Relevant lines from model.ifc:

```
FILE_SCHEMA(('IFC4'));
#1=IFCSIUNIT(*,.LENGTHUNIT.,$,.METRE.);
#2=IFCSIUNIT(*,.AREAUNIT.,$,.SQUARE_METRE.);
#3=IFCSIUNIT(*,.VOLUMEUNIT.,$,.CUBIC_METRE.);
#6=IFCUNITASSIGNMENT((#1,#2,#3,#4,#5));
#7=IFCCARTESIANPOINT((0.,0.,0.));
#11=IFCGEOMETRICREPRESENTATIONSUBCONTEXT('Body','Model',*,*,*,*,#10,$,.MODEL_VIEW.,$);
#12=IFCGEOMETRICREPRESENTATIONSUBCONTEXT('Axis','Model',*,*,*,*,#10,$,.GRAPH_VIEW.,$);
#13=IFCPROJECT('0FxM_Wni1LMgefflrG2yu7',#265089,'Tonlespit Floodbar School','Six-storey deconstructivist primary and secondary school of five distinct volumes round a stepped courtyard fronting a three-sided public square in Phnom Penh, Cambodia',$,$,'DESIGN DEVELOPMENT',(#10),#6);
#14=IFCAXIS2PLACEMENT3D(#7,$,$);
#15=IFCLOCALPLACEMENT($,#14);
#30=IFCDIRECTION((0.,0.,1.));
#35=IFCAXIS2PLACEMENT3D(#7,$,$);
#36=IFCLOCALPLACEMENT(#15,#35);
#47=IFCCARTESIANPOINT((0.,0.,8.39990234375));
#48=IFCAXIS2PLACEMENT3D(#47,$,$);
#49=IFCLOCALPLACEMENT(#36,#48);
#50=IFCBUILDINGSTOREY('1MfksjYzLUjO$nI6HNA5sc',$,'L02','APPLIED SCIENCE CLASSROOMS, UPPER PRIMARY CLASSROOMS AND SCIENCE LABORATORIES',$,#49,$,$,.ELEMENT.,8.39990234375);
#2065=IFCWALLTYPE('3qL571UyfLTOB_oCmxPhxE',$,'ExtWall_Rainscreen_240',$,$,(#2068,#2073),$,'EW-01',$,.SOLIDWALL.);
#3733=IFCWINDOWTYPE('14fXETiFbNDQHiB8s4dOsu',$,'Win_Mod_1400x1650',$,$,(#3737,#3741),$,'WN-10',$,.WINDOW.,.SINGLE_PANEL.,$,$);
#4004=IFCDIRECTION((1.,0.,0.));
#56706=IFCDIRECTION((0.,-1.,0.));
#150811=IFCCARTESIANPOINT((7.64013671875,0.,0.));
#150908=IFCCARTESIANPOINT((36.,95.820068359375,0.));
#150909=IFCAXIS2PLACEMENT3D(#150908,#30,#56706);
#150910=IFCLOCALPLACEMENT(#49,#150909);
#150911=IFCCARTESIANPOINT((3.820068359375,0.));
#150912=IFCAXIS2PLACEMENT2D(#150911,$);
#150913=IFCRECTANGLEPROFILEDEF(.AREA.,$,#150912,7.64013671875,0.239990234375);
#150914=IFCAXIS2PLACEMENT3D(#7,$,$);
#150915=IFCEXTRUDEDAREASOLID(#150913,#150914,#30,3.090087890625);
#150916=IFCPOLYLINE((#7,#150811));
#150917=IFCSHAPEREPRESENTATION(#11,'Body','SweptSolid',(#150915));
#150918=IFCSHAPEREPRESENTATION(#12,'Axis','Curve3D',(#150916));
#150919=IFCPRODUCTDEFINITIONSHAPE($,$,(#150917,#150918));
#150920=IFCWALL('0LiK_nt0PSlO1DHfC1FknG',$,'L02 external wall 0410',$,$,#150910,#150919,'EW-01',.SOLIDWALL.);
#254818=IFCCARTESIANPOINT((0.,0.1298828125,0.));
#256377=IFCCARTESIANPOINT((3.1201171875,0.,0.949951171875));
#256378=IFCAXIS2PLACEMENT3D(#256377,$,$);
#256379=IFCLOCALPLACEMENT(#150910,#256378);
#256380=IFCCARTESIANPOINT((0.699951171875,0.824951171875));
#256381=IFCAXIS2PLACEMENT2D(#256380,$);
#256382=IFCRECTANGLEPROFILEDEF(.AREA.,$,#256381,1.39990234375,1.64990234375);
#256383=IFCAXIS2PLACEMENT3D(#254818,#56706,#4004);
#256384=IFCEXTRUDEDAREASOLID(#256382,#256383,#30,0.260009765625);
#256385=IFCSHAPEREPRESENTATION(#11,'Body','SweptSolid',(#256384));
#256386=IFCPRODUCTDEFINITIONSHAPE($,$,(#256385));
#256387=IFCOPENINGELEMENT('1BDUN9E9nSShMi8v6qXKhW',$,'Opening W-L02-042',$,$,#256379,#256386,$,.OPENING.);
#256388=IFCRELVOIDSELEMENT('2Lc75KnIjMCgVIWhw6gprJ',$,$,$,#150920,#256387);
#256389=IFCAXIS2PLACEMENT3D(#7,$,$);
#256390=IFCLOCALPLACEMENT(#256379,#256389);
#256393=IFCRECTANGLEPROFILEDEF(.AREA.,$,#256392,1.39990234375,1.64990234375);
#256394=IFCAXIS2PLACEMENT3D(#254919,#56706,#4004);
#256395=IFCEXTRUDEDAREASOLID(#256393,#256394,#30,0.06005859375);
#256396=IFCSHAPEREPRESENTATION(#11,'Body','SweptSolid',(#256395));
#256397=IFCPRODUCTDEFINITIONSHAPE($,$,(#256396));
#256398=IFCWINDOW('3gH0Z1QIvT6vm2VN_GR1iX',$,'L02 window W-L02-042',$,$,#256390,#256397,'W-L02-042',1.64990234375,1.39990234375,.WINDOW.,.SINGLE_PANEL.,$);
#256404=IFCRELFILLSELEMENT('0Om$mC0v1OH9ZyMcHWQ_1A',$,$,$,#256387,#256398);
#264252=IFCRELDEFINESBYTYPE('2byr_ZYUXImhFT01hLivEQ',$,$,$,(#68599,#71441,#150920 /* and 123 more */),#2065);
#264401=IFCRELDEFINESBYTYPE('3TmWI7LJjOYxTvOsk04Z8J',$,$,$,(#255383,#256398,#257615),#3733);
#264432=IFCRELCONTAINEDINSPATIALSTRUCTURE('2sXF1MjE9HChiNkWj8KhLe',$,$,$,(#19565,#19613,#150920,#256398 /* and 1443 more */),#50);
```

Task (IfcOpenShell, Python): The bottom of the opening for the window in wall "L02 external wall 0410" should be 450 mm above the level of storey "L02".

```python
import numpy as np
import ifcopenshell
import ifcopenshell.api.geometry
import ifcopenshell.geom
import ifcopenshell.util.element
import ifcopenshell.util.placement
import ifcopenshell.util.shape
import ifcopenshell.util.unit

model = ifcopenshell.open("model.ifc")
unit_scale = ifcopenshell.util.unit.calculate_unit_scale(model)

window = model.by_guid("3gH0Z1QIvT6vm2VN_GR1iX")
opening = window.FillsVoids[0].RelatingOpeningElement
storey = ifcopenshell.util.element.get_container(window, ifc_class="IfcBuildingStorey")
level = ifcopenshell.util.placement.get_local_placement(storey.ObjectPlacement)[2, 3]

# The opening's origin need not be at the sill, so measure its lowest point.
shape = ifcopenshell.geom.create_shape(ifcopenshell.geom.settings(), opening)
bottom = ifcopenshell.util.shape.get_shape_bottom_elevation(shape, shape.geometry) / unit_scale
dz = level + 0.45 / unit_scale - bottom

shift = np.array([0.0, 0.0, dz])
# The window is placed relative to its opening, so it follows when the opening moves.
matrix = ifcopenshell.util.placement.get_local_placement(opening.ObjectPlacement)
matrix[:3, 3] += shift
ifcopenshell.api.geometry.edit_object_placement(
    model, product=opening, matrix=matrix, is_si=False, should_transform_children=True
)

print(f"moved by {dz * unit_scale:+.3f} m")

model.write("model_updated.ifc")
```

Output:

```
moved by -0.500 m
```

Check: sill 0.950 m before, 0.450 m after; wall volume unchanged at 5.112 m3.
